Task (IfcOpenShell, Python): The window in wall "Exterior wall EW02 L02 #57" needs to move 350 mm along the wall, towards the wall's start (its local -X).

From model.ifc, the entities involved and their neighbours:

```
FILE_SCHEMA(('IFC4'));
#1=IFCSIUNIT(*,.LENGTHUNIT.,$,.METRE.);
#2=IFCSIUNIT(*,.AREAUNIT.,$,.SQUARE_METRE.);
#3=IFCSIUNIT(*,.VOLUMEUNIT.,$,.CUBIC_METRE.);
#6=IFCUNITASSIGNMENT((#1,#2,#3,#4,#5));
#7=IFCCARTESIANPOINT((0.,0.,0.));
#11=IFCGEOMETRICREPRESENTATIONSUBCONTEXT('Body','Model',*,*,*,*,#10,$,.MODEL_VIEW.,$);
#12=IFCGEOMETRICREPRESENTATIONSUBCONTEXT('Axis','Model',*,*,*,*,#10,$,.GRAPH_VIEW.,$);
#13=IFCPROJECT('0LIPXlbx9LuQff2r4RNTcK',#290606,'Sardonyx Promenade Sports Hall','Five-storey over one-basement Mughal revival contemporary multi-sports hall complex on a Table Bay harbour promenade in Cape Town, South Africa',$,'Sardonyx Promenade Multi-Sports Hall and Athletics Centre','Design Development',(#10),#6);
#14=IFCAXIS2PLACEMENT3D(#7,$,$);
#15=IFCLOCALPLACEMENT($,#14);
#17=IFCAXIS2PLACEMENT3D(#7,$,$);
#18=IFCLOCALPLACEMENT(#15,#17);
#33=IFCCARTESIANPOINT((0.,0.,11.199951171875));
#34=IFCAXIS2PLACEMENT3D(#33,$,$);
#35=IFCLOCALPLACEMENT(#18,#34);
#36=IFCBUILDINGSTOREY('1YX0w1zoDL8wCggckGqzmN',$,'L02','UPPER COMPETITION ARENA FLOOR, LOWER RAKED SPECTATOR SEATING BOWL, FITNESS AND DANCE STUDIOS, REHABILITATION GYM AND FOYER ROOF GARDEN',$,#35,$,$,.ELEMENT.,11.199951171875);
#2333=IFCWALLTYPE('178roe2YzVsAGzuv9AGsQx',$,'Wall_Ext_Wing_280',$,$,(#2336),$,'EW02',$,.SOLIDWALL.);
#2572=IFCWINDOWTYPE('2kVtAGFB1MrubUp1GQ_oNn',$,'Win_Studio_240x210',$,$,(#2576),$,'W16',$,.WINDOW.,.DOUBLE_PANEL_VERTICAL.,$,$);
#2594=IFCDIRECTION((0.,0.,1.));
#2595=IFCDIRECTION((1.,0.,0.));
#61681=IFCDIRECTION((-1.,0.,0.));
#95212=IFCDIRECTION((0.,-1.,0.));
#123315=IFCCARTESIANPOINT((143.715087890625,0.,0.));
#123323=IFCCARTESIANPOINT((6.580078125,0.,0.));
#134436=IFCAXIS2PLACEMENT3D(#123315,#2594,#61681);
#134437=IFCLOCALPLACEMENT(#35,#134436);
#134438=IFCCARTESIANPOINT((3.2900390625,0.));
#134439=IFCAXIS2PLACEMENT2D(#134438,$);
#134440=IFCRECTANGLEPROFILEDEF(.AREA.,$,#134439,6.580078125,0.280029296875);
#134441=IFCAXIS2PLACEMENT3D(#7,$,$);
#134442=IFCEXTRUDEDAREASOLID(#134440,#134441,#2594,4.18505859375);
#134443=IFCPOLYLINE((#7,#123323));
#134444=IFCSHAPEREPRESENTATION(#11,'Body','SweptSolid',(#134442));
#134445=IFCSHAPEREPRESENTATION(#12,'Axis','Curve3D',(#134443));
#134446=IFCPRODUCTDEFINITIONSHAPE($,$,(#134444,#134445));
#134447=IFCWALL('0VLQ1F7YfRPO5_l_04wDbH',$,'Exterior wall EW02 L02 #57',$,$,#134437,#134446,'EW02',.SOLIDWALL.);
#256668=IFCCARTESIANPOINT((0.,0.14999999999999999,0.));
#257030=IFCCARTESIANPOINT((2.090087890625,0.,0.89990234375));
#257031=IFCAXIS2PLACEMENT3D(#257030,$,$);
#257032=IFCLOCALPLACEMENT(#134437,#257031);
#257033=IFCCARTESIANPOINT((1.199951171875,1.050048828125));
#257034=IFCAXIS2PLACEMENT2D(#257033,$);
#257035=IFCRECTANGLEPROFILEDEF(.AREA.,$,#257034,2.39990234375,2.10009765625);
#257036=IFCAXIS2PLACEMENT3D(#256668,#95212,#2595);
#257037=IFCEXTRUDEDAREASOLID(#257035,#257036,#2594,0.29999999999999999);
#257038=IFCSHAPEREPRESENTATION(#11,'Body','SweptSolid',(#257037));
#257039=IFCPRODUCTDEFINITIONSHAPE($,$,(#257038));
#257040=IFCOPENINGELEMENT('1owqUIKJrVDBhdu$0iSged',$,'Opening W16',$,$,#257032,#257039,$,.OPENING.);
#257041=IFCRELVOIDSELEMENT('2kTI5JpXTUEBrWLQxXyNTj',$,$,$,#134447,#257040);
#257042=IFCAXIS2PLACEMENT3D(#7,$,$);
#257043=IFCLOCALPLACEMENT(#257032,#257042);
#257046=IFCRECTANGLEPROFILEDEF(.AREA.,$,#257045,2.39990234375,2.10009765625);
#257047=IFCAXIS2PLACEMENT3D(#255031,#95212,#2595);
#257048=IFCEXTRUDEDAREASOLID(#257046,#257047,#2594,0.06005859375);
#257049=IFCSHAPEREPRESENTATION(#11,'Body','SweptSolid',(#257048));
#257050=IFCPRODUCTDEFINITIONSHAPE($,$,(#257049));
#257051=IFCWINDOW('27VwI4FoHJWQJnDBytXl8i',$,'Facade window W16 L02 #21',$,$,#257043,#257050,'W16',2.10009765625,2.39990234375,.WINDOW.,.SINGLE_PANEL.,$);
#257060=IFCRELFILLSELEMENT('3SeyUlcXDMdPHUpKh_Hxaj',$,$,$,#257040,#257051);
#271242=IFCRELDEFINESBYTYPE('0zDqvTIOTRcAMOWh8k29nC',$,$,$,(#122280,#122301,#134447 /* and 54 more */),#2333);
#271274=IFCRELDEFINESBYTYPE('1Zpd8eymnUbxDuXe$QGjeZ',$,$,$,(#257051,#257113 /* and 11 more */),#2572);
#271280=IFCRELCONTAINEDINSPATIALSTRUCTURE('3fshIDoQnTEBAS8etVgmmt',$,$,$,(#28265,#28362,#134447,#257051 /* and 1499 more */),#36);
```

```python
import ifcopenshell
import ifcopenshell.api.geometry
import ifcopenshell.util.placement

model = ifcopenshell.open("model.ifc")

window = model.by_guid("27VwI4FoHJWQJnDBytXl8i")
opening = window.FillsVoids[0].RelatingOpeningElement
wall = opening.VoidsElements[0].RelatingBuildingElement

wall_matrix = ifcopenshell.util.placement.get_local_placement(wall.ObjectPlacement)
shift = wall_matrix[:3, 0] * -0.35
before = ifcopenshell.util.placement.get_local_placement(window.ObjectPlacement)[:3, 3].copy()

# The window is placed relative to its opening, so it follows when the opening moves.
matrix = ifcopenshell.util.placement.get_local_placement(opening.ObjectPlacement)
matrix[:3, 3] += shift
ifcopenshell.api.geometry.edit_object_placement(
    model, product=opening, matrix=matrix, is_si=False, should_transform_children=True
)

after = ifcopenshell.util.placement.get_local_placement(window.ObjectPlacement)[:3, 3]
print("window moved by", (after - before).round(3) + 0.0)

model.write("model_updated.ifc")
```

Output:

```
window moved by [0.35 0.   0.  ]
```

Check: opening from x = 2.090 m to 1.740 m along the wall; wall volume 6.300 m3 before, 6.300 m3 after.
